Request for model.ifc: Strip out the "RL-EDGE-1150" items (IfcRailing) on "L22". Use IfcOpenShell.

First a look at what the model holds.

```python
import ifcopenshell
import ifcopenshell.util.element

model = ifcopenshell.open("model.ifc")
print(model.schema)
storey = next(s for s in model.by_type("IfcBuildingStorey") if s.Name == "L22")
railings = [e for e in ifcopenshell.util.element.get_decomposition(storey) if e.is_a("IfcRailing")]
seen = {}
for e in railings:
    element_type = ifcopenshell.util.element.get_type(e)
    name = element_type.Name if element_type not in (None, e) else None
    seen[name] = seen.get(name, 0) + 1
for name, count in sorted(seen.items(), key=str):
    print(count, "x", name)
```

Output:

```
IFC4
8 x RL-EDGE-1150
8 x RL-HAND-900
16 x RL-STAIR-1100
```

```python
import ifcopenshell
import ifcopenshell.api.root
import ifcopenshell.util.element

model = ifcopenshell.open("model.ifc")

storey = next(s for s in model.by_type("IfcBuildingStorey") if s.Name == "L22")
railings = [e for e in ifcopenshell.util.element.get_decomposition(storey) if e.is_a("IfcRailing")]
targets = [e for e in railings if (t := ifcopenshell.util.element.get_type(e)) not in (None, e) and t.Name == "RL-EDGE-1150"]

for e in targets:
    ifcopenshell.api.root.remove_product(model, product=e)
print(len(targets), "removed")

model.write("model_v2.ifc")
```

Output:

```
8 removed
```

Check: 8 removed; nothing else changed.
